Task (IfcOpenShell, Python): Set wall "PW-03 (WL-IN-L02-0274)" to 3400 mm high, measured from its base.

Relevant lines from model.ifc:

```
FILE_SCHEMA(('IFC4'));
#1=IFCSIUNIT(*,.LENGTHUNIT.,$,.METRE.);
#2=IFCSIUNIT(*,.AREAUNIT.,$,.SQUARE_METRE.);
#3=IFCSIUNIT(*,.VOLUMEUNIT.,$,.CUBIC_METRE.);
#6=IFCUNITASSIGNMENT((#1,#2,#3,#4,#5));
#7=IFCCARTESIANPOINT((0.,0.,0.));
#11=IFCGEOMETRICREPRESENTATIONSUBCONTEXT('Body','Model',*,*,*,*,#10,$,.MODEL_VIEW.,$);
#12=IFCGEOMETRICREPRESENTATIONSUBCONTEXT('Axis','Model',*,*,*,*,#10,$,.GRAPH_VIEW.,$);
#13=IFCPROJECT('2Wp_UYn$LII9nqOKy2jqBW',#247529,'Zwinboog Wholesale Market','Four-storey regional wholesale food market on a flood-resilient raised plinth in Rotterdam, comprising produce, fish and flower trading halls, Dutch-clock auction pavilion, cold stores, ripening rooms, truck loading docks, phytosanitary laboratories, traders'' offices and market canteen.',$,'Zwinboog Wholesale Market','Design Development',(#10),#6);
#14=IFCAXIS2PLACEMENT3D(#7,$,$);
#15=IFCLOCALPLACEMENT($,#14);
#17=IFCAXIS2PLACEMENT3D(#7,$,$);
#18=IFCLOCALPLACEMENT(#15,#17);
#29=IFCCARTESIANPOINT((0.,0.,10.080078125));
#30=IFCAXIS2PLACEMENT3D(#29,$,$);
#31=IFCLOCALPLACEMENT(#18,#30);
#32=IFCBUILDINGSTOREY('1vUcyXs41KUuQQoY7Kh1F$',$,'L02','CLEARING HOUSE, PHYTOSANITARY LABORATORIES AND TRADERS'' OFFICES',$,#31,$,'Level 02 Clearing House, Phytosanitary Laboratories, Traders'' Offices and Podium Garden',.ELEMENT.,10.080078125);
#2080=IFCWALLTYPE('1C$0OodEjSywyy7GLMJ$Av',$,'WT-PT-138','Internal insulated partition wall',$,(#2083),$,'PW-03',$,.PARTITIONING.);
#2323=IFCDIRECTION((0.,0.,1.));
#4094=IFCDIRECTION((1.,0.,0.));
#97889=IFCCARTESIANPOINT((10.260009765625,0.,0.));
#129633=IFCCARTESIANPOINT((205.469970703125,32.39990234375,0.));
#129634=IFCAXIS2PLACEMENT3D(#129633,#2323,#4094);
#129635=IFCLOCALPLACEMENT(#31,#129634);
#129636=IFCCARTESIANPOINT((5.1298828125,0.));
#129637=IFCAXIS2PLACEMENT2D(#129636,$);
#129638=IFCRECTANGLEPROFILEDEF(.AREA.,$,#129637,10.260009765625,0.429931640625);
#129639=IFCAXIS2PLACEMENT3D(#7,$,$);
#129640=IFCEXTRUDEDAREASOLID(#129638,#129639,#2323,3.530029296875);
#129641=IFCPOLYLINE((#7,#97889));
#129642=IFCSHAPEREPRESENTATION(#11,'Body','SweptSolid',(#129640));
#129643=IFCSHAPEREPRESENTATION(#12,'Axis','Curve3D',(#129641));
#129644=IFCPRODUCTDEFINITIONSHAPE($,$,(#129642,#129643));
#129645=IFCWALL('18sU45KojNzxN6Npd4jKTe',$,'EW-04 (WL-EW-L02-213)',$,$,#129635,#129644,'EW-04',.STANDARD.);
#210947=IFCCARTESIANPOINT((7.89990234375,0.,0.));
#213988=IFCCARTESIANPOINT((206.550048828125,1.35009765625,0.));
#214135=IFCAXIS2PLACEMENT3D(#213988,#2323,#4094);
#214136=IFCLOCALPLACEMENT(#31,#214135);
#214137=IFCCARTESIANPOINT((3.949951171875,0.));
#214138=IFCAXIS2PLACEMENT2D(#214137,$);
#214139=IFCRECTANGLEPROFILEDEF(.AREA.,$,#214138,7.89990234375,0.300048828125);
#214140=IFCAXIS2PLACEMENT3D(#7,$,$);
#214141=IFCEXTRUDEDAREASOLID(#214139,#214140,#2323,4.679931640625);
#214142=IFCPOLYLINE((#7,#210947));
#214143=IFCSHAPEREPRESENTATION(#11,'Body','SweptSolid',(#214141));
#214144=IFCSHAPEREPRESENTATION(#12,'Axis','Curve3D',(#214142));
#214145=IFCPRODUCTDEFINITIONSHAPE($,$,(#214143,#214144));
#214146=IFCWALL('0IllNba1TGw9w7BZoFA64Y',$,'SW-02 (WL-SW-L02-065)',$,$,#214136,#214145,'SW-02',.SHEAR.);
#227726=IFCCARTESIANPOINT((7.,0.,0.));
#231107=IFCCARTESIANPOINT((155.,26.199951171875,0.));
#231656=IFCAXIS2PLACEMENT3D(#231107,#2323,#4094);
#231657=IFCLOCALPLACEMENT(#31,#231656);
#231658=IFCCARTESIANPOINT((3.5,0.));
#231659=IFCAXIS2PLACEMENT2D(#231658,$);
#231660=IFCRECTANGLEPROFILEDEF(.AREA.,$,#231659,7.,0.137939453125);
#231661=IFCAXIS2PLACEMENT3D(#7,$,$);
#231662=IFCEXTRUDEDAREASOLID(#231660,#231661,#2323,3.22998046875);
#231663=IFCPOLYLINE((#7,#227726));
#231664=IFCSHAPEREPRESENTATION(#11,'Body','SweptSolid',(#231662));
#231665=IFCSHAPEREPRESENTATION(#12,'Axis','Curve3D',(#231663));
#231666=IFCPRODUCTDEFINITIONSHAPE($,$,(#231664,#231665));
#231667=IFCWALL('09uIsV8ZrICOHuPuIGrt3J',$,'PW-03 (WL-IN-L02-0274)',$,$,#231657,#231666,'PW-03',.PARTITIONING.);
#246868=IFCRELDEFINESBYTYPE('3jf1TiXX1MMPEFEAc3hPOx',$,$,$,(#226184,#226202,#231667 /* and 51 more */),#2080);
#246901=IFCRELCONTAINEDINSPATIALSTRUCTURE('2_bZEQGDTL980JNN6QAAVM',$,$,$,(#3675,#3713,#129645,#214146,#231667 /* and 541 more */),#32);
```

```python
import ifcopenshell
import ifcopenshell.geom
import ifcopenshell.util.representation
import ifcopenshell.util.shape
import ifcopenshell.util.unit

model = ifcopenshell.open("model.ifc")
unit_scale = ifcopenshell.util.unit.calculate_unit_scale(model)
settings = ifcopenshell.geom.settings()


def volume(element):
    """Net volume in cubic metres, openings subtracted."""
    shape = ifcopenshell.geom.create_shape(settings, element)
    return ifcopenshell.util.shape.get_volume(shape.geometry)


wall = model.by_guid("09uIsV8ZrICOHuPuIGrt3J")
before = volume(wall)

body = ifcopenshell.util.representation.get_representation(wall, "Model", "Body")
solid = body.Items[0]
old_height = solid.Depth
solid.Depth = 3.4 / unit_scale
after = volume(wall)

print(f"height {old_height:g} -> {solid.Depth:g}, volume {before:.3f} -> {after:.3f} m3")

model.write("model_rev.ifc")
```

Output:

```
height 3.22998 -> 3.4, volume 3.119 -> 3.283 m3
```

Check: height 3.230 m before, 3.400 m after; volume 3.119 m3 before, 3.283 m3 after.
